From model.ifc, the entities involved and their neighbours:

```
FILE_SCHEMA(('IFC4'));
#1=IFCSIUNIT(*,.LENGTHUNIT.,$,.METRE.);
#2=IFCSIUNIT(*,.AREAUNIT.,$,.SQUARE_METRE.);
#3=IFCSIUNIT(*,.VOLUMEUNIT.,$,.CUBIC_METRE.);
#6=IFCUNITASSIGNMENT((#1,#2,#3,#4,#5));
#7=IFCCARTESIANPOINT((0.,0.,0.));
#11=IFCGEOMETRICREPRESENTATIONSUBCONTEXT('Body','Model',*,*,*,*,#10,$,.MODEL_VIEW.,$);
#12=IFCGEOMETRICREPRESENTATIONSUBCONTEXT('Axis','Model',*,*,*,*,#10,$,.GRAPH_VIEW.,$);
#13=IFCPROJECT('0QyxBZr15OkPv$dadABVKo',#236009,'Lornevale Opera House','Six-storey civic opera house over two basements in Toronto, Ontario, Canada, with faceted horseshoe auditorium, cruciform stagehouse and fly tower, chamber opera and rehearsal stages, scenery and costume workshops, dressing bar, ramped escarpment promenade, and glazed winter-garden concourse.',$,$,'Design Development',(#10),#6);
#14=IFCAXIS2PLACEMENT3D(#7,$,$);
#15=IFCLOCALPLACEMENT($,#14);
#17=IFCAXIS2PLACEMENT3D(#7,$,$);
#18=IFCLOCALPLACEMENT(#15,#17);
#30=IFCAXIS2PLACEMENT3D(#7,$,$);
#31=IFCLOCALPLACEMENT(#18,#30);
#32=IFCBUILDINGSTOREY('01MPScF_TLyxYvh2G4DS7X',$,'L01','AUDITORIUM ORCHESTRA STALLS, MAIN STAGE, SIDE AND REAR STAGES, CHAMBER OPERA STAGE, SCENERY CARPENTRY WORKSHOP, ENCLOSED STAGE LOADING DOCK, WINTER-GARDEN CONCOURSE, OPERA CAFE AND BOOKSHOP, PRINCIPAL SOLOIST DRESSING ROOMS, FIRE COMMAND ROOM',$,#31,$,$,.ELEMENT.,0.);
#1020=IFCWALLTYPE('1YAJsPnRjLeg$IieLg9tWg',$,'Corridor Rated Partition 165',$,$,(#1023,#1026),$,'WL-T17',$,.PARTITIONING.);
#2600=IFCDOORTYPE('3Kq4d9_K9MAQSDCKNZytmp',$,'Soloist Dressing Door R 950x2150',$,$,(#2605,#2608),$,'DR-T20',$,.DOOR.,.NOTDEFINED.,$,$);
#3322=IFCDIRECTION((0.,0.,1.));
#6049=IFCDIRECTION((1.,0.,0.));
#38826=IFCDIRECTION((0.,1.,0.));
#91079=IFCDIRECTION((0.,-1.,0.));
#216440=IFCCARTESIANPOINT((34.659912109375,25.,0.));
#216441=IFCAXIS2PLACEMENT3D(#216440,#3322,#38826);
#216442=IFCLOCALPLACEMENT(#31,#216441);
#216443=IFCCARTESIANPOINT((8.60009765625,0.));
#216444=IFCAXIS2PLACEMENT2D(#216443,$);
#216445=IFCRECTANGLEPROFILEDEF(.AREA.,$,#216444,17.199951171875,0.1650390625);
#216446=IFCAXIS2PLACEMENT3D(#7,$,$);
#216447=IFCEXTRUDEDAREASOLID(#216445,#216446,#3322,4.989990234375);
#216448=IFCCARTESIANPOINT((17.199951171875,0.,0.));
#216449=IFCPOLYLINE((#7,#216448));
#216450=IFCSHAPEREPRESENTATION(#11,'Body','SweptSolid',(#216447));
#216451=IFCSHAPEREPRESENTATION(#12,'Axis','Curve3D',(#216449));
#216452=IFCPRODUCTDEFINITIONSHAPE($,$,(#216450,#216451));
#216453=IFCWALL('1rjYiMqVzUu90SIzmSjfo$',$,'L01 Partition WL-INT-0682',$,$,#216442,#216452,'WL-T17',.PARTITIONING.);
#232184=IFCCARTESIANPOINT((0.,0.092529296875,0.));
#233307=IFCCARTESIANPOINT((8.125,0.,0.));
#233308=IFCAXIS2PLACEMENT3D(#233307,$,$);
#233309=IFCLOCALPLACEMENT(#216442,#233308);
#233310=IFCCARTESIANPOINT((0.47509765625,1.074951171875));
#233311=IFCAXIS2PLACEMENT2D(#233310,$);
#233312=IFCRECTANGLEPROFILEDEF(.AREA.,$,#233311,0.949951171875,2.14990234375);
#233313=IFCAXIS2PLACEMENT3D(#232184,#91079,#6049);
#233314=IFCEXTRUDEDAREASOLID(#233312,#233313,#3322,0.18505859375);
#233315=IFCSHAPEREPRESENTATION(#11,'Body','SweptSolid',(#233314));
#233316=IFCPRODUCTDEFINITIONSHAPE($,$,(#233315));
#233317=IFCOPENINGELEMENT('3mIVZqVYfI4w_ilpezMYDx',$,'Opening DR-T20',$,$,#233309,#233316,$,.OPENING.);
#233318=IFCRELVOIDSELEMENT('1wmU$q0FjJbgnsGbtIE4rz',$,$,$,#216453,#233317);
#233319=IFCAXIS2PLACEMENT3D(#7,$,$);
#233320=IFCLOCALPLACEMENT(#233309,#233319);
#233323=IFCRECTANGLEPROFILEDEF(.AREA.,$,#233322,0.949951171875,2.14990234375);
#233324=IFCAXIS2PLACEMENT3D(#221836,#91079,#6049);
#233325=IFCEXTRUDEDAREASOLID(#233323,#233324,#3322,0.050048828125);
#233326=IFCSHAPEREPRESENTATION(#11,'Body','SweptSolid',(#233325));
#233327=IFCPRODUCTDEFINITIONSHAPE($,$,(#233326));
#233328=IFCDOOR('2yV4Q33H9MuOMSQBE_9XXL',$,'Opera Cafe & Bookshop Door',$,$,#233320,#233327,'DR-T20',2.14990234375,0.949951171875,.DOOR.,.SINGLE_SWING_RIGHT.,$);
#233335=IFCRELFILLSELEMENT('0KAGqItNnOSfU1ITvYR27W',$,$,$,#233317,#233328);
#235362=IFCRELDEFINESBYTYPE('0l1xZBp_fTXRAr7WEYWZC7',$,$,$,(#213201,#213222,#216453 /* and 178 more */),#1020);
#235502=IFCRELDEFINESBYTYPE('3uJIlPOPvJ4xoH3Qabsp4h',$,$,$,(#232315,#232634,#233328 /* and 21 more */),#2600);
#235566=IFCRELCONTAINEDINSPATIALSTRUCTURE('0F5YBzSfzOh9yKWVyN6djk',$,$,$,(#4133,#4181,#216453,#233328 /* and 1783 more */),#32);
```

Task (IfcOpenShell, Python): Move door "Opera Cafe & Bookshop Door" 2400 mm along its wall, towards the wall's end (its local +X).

```python
import ifcopenshell
import ifcopenshell.api.geometry
import ifcopenshell.util.placement
import ifcopenshell.util.unit

model = ifcopenshell.open("model.ifc")
unit_scale = ifcopenshell.util.unit.calculate_unit_scale(model)

door = model.by_guid("2yV4Q33H9MuOMSQBE_9XXL")
opening = door.FillsVoids[0].RelatingOpeningElement
wall = opening.VoidsElements[0].RelatingBuildingElement

wall_matrix = ifcopenshell.util.placement.get_local_placement(wall.ObjectPlacement)
shift = wall_matrix[:3, 0] * 2.4 / unit_scale
before = ifcopenshell.util.placement.get_local_placement(door.ObjectPlacement)[:3, 3].copy()

# The door is placed relative to its opening, so it follows when the opening moves.
matrix = ifcopenshell.util.placement.get_local_placement(opening.ObjectPlacement)
matrix[:3, 3] += shift
ifcopenshell.api.geometry.edit_object_placement(
    model, product=opening, matrix=matrix, is_si=False, should_transform_children=True
)

after = ifcopenshell.util.placement.get_local_placement(door.ObjectPlacement)[:3, 3]
print("door moved by", (after - before).round(3) + 0.0)

model.write("model_edited.ifc")
```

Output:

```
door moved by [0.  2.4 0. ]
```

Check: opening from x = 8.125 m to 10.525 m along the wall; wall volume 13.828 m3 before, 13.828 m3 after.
